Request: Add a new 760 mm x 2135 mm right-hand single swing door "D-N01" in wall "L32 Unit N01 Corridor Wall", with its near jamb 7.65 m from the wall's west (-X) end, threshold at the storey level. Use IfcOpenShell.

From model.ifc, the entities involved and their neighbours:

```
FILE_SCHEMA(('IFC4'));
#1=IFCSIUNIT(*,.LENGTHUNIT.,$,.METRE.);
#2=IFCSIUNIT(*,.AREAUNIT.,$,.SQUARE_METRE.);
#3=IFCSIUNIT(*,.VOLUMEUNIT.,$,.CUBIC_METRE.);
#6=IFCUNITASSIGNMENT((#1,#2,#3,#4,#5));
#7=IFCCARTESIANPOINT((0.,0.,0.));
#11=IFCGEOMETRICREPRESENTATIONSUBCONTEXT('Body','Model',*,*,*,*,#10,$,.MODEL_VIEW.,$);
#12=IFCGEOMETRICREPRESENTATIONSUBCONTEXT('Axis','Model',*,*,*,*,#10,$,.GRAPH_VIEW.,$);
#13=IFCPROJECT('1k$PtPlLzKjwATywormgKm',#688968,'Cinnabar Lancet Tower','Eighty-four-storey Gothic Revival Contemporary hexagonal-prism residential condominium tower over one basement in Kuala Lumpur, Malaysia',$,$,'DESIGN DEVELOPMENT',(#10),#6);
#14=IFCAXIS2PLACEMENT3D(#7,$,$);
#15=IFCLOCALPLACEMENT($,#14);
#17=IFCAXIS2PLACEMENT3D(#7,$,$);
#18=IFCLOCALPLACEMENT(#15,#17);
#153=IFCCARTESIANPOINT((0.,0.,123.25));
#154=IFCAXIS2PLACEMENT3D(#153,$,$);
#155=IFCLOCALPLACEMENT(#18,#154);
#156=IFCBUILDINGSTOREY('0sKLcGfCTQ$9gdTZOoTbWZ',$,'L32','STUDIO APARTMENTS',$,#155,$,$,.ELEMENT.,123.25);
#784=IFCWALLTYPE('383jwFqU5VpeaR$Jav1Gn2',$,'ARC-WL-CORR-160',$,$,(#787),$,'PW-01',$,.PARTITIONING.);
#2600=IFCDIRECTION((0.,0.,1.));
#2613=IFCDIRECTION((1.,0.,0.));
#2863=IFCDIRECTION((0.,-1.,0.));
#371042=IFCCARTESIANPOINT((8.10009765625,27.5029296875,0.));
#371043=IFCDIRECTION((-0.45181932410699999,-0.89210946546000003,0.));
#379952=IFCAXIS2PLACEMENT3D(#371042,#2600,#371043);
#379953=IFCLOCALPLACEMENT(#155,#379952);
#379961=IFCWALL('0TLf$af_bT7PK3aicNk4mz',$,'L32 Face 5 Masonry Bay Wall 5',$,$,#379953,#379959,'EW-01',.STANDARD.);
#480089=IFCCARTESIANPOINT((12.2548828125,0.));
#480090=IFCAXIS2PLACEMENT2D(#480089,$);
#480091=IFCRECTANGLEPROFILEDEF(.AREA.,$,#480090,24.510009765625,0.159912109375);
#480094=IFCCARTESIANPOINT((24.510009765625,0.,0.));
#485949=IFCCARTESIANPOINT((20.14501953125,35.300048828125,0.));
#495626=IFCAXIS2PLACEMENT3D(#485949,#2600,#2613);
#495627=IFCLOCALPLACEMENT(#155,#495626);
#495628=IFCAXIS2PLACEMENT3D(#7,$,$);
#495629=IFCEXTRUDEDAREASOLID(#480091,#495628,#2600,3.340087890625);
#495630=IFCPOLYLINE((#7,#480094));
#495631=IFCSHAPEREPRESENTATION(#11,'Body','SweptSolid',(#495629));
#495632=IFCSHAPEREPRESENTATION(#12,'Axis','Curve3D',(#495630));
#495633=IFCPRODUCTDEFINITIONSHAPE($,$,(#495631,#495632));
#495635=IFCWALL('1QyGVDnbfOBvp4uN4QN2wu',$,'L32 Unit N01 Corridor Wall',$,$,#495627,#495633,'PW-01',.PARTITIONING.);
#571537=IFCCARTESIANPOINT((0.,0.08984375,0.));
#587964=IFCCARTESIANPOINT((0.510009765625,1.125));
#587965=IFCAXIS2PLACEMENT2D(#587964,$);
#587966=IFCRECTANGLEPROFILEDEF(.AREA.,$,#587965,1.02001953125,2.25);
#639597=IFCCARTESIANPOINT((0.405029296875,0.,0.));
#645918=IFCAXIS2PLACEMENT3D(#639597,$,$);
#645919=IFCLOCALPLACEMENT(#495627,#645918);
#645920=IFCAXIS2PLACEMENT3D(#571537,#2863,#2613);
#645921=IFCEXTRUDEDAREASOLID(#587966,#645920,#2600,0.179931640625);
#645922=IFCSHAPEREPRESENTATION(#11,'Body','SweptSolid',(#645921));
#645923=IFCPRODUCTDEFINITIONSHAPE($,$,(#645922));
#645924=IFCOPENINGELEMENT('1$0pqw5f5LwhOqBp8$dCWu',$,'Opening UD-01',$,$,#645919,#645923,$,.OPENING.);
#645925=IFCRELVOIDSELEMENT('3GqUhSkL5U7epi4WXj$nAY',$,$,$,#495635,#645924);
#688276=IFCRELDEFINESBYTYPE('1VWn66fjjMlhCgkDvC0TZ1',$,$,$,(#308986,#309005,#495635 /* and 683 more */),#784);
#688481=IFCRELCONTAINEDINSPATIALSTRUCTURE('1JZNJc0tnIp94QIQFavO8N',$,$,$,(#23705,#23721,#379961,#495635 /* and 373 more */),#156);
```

```python
import numpy as np
import ifcopenshell
import ifcopenshell.api.feature
import ifcopenshell.api.geometry
import ifcopenshell.api.root
import ifcopenshell.api.spatial
import ifcopenshell.geom
import ifcopenshell.util.element
import ifcopenshell.util.placement
import ifcopenshell.util.representation
import ifcopenshell.util.shape
import ifcopenshell.util.unit

model = ifcopenshell.open("model.ifc")
unit_scale = ifcopenshell.util.unit.calculate_unit_scale(model)
settings = ifcopenshell.geom.settings()


def volume(element):
    """Net volume in cubic metres, openings subtracted."""
    shape = ifcopenshell.geom.create_shape(settings, element)
    return ifcopenshell.util.shape.get_volume(shape.geometry)


wall = model.by_guid("1QyGVDnbfOBvp4uN4QN2wu")
storey = ifcopenshell.util.element.get_container(wall, ifc_class="IfcBuildingStorey")
context = ifcopenshell.util.representation.get_context(model, "Model", "Body", "MODEL_VIEW")
before = volume(wall)

width, height, from_end, sill = 0.76, 2.135, 7.65, 0.0  # metres

# The wall runs along its own X axis, and the end named is its -X end.
wall_shape = ifcopenshell.geom.create_shape(settings, wall)
x, y, z = ifcopenshell.util.shape.get_vertices(wall_shape.geometry).T
start = x.min() + from_end
face, thickness = float(y.min()), float(y.max() - y.min())
wall_matrix = ifcopenshell.util.placement.get_local_placement(wall.ObjectPlacement)
level = ifcopenshell.util.placement.get_local_placement(storey.ObjectPlacement)[2, 3]


def in_wall(x, y):
    """Placement at x, y metres in the wall's axes, at sill height."""
    matrix = wall_matrix.copy()
    matrix[:, 3] = wall_matrix @ np.array([x / unit_scale, y / unit_scale, 0.0, 1.0])
    matrix[2, 3] = level + sill / unit_scale
    return matrix


# Opening: a box that overshoots both wall faces by 50 mm.
opening = ifcopenshell.api.root.create_entity(model, ifc_class="IfcOpeningElement", predefined_type="OPENING")
box = ifcopenshell.api.geometry.add_wall_representation(
    model, context=context, length=width, height=height, thickness=thickness + 0.1
)
ifcopenshell.api.geometry.assign_representation(model, product=opening, representation=box)
ifcopenshell.api.geometry.edit_object_placement(model, product=opening, matrix=in_wall(start, face - 0.05), is_si=False)
ifcopenshell.api.feature.add_feature(model, feature=opening, element=wall)

door = ifcopenshell.api.root.create_entity(model, ifc_class="IfcDoor", name="D-N01", predefined_type="DOOR")
door.OverallWidth, door.OverallHeight = width / unit_scale, height / unit_scale
door.OperationType = "SINGLE_SWING_RIGHT"
body = ifcopenshell.api.geometry.add_door_representation(
    model,
    context=context,
    overall_width=door.OverallWidth,
    overall_height=door.OverallHeight,
    operation_type="SINGLE_SWING_RIGHT",
    lining_properties={"LiningDepth": thickness / unit_scale, "ThresholdDepth": thickness / unit_scale},
)
ifcopenshell.api.geometry.assign_representation(model, product=door, representation=body)
ifcopenshell.api.spatial.assign_container(model, products=[door], relating_structure=storey)
ifcopenshell.api.feature.add_filling(model, opening=opening, element=door)

# The lining spans the wall, so the door starts at the wall face.
ifcopenshell.api.geometry.edit_object_placement(model, product=door, matrix=in_wall(start, face), is_si=False)

after = volume(wall)

print(f"wall volume {before:.3f} -> {after:.3f} m3")

model.write("model-out.ifc")
```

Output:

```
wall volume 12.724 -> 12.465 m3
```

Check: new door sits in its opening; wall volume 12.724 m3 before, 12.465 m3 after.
